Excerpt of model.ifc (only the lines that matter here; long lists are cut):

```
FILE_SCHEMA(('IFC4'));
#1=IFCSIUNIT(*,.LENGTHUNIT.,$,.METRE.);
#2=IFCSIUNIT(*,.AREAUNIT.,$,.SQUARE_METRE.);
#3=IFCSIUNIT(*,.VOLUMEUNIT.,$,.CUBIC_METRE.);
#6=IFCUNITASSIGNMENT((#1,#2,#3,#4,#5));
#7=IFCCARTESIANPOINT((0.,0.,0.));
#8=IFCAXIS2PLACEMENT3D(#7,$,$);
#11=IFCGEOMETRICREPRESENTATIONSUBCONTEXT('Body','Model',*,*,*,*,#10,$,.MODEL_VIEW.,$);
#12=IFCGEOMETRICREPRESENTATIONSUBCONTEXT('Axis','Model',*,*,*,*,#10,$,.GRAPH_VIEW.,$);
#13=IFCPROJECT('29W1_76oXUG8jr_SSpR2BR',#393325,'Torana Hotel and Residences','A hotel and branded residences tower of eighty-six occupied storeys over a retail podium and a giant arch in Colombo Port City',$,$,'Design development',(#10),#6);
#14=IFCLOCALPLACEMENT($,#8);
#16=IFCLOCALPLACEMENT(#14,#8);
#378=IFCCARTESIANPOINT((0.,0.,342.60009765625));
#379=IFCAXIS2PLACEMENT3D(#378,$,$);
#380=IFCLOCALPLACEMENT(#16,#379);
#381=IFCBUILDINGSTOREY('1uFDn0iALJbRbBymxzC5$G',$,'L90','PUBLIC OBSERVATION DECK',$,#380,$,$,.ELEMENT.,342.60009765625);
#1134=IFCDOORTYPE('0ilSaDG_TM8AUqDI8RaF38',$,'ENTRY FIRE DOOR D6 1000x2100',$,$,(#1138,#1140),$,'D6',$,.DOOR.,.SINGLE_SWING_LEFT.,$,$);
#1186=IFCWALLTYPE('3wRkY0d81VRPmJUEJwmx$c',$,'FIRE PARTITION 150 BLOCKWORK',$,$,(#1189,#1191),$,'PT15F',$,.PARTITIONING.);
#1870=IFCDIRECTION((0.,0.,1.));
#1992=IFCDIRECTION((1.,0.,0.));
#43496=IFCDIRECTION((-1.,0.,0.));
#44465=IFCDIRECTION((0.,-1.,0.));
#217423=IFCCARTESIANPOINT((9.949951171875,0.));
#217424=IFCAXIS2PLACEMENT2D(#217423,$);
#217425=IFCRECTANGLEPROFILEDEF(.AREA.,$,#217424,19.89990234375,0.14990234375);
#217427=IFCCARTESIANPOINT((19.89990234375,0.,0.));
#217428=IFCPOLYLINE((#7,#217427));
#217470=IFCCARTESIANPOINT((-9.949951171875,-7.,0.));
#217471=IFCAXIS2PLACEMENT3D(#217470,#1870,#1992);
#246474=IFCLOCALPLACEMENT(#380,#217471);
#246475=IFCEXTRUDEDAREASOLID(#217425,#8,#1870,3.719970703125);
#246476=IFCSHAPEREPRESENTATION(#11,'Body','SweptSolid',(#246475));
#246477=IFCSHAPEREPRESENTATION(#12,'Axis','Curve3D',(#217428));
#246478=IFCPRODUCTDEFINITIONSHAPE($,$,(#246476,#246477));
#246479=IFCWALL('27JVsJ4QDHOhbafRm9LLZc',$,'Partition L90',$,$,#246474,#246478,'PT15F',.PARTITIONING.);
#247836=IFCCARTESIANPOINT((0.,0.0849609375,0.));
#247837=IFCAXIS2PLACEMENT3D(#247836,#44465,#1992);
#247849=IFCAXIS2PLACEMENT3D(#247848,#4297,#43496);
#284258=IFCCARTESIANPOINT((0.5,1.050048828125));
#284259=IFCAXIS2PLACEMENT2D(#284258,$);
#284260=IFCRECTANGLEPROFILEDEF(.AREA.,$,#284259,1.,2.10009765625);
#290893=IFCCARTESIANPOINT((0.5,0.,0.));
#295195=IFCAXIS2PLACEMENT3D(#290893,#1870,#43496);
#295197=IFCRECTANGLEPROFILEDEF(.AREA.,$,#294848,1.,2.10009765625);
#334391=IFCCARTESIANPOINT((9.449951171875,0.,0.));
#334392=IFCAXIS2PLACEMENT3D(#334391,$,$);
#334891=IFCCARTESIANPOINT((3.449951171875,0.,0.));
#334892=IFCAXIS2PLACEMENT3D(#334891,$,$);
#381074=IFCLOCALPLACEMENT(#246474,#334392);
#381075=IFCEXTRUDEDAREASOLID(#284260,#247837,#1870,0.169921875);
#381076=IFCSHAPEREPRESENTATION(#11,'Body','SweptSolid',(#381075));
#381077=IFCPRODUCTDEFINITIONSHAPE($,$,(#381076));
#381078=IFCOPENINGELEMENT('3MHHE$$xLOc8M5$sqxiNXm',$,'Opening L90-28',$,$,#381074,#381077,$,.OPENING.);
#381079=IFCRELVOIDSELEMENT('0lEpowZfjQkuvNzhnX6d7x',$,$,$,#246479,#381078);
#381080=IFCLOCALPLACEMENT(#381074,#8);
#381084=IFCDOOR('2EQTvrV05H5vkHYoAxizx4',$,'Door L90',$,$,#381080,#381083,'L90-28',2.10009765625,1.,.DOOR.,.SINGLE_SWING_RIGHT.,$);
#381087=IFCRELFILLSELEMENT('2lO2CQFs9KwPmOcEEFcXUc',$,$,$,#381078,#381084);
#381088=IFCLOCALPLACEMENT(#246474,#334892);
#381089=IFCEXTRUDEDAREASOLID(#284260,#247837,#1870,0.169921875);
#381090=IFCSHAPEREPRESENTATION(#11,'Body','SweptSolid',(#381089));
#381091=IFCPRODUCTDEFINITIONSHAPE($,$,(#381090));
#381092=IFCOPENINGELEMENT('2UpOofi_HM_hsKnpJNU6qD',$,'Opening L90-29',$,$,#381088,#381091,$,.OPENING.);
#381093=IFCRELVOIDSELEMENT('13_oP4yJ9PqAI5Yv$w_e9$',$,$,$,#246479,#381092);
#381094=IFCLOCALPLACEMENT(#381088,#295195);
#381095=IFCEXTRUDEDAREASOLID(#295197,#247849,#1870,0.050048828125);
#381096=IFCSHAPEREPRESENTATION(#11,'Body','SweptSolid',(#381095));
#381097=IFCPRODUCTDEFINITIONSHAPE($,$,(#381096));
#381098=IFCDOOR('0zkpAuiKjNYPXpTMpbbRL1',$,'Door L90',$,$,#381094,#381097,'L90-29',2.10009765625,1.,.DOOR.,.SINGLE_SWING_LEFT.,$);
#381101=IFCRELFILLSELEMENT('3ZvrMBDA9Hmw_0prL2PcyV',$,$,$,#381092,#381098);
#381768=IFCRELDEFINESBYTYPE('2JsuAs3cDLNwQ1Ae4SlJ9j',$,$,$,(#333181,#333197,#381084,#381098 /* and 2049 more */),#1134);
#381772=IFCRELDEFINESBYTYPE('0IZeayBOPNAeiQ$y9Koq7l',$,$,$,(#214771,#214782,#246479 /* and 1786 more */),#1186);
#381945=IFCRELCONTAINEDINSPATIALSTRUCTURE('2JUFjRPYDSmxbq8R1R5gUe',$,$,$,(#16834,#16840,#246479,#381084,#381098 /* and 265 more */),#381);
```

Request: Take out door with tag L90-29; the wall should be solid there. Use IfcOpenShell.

```python
import ifcopenshell
import ifcopenshell.api.feature
import ifcopenshell.api.root
import ifcopenshell.geom
import ifcopenshell.util.shape

model = ifcopenshell.open("model.ifc")
settings = ifcopenshell.geom.settings()


def volume(element):
    """Net volume in cubic metres, openings subtracted."""
    shape = ifcopenshell.geom.create_shape(settings, element)
    return ifcopenshell.util.shape.get_volume(shape.geometry)


door = model.by_id(381098)
opening = door.FillsVoids[0].RelatingOpeningElement
wall = opening.VoidsElements[0].RelatingBuildingElement
before = volume(wall)

ifcopenshell.api.root.remove_product(model, product=door)
ifcopenshell.api.feature.remove_feature(model, feature=opening)

after = volume(wall)

print(f"wall volume {before:.3f} -> {after:.3f} m3")

model.write("model_rev.ifc")
```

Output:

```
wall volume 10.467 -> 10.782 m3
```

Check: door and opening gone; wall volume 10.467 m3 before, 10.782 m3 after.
